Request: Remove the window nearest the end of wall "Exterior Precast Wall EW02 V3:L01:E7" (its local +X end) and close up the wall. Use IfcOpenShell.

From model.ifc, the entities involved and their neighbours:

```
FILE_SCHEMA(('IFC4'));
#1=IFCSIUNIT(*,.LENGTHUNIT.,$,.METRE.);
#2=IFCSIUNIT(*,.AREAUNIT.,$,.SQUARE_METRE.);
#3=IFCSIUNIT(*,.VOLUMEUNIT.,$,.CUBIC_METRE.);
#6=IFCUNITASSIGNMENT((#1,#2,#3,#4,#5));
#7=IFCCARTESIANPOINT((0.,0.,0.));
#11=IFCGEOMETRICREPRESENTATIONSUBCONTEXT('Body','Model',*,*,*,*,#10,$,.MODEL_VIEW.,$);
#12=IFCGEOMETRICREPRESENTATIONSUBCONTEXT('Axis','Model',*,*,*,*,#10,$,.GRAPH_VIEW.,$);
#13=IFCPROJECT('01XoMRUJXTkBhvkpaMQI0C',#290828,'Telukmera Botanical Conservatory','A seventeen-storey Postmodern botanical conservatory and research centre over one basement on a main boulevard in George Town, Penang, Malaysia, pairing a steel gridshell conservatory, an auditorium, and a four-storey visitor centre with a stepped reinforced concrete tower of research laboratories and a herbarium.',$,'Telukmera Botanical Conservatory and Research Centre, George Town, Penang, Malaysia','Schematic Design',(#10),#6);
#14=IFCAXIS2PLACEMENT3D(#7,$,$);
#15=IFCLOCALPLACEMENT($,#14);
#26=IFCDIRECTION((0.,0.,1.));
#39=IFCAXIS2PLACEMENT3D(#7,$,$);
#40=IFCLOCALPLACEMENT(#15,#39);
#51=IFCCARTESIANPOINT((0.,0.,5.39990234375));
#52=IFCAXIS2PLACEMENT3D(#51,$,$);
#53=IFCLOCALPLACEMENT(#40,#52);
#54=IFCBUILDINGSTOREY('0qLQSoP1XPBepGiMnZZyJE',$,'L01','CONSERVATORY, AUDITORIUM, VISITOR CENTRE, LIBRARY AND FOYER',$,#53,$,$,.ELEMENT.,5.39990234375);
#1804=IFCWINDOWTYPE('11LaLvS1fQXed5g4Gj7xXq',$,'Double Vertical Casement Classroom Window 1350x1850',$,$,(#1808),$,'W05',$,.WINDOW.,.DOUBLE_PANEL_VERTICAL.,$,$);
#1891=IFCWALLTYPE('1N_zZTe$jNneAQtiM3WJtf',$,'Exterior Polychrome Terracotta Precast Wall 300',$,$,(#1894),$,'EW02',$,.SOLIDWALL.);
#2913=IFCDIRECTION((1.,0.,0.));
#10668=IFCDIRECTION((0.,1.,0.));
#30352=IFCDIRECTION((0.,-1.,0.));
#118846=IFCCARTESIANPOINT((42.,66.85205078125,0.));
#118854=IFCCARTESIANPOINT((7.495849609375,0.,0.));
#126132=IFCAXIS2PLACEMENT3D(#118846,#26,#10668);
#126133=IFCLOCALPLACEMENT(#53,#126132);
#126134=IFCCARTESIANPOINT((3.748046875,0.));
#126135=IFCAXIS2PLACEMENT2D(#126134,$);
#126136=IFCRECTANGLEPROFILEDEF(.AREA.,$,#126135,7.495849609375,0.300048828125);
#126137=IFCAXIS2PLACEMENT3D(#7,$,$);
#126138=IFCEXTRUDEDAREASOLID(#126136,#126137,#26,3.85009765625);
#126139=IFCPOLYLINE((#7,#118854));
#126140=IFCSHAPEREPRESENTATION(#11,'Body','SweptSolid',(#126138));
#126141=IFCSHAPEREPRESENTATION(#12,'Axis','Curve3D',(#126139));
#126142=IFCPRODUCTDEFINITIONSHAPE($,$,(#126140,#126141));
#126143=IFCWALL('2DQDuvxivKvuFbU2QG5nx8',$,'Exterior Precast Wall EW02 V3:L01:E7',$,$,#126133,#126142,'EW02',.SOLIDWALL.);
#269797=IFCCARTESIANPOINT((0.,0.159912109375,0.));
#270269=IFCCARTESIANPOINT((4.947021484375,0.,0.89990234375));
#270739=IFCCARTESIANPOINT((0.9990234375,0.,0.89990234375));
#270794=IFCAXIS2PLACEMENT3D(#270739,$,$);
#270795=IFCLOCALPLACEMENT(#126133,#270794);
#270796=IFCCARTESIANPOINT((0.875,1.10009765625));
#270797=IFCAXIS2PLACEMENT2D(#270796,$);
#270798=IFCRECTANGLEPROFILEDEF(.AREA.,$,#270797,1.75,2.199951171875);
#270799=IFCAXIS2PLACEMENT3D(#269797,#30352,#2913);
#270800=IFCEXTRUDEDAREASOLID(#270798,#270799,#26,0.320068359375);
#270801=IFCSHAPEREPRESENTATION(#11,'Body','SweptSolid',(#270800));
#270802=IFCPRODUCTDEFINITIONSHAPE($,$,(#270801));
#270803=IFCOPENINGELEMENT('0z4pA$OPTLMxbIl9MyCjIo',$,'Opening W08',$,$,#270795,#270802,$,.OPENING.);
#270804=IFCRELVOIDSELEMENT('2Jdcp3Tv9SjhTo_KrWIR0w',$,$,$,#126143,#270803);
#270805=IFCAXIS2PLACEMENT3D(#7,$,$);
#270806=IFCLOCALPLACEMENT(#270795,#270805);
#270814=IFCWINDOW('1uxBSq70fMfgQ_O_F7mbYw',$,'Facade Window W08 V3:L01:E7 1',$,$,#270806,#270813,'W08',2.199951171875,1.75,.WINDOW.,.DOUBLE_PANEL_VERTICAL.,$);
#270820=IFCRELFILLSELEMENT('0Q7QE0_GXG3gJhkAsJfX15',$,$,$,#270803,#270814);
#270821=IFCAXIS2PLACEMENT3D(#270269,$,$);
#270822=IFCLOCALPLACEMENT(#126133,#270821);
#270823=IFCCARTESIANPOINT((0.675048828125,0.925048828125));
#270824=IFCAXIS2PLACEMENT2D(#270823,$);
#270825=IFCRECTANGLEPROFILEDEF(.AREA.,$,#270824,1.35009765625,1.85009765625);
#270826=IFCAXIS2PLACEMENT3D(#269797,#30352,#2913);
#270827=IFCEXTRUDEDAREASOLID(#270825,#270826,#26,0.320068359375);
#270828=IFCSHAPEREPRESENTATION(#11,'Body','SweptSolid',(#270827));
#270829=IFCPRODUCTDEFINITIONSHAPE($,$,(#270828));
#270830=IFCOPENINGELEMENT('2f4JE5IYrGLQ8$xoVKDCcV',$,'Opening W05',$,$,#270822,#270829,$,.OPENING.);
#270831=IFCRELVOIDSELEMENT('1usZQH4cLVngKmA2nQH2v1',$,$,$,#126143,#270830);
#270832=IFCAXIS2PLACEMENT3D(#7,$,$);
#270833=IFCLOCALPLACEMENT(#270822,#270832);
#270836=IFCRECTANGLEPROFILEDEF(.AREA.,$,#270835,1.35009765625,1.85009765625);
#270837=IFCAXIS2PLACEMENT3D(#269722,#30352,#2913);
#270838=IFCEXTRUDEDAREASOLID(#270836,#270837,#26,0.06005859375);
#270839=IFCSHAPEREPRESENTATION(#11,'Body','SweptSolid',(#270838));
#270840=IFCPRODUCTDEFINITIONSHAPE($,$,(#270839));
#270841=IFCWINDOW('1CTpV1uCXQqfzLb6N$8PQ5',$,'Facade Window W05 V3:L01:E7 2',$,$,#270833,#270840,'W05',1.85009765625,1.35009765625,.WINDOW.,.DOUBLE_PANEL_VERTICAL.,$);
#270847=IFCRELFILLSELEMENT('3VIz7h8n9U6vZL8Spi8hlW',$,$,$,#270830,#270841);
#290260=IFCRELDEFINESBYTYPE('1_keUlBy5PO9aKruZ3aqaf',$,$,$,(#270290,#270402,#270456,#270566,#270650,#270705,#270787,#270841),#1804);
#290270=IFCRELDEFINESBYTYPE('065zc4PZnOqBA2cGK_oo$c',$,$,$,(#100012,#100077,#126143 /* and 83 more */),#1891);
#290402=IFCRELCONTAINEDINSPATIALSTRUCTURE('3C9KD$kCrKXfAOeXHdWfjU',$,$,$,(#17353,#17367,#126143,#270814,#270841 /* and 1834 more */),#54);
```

```python
import ifcopenshell
import ifcopenshell.api.feature
import ifcopenshell.api.root
import ifcopenshell.geom
import ifcopenshell.util.shape

model = ifcopenshell.open("model.ifc")
settings = ifcopenshell.geom.settings()


def volume(element):
    """Net volume in cubic metres, openings subtracted."""
    shape = ifcopenshell.geom.create_shape(settings, element)
    return ifcopenshell.util.shape.get_volume(shape.geometry)


window = model.by_id(270841)
opening = window.FillsVoids[0].RelatingOpeningElement
wall = opening.VoidsElements[0].RelatingBuildingElement
before = volume(wall)

ifcopenshell.api.root.remove_product(model, product=window)
ifcopenshell.api.feature.remove_feature(model, feature=opening)

after = volume(wall)

print(f"wall volume {before:.3f} -> {after:.3f} m3")

model.write("model_updated.ifc")
```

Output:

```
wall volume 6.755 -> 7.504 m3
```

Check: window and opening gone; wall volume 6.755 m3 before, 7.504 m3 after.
